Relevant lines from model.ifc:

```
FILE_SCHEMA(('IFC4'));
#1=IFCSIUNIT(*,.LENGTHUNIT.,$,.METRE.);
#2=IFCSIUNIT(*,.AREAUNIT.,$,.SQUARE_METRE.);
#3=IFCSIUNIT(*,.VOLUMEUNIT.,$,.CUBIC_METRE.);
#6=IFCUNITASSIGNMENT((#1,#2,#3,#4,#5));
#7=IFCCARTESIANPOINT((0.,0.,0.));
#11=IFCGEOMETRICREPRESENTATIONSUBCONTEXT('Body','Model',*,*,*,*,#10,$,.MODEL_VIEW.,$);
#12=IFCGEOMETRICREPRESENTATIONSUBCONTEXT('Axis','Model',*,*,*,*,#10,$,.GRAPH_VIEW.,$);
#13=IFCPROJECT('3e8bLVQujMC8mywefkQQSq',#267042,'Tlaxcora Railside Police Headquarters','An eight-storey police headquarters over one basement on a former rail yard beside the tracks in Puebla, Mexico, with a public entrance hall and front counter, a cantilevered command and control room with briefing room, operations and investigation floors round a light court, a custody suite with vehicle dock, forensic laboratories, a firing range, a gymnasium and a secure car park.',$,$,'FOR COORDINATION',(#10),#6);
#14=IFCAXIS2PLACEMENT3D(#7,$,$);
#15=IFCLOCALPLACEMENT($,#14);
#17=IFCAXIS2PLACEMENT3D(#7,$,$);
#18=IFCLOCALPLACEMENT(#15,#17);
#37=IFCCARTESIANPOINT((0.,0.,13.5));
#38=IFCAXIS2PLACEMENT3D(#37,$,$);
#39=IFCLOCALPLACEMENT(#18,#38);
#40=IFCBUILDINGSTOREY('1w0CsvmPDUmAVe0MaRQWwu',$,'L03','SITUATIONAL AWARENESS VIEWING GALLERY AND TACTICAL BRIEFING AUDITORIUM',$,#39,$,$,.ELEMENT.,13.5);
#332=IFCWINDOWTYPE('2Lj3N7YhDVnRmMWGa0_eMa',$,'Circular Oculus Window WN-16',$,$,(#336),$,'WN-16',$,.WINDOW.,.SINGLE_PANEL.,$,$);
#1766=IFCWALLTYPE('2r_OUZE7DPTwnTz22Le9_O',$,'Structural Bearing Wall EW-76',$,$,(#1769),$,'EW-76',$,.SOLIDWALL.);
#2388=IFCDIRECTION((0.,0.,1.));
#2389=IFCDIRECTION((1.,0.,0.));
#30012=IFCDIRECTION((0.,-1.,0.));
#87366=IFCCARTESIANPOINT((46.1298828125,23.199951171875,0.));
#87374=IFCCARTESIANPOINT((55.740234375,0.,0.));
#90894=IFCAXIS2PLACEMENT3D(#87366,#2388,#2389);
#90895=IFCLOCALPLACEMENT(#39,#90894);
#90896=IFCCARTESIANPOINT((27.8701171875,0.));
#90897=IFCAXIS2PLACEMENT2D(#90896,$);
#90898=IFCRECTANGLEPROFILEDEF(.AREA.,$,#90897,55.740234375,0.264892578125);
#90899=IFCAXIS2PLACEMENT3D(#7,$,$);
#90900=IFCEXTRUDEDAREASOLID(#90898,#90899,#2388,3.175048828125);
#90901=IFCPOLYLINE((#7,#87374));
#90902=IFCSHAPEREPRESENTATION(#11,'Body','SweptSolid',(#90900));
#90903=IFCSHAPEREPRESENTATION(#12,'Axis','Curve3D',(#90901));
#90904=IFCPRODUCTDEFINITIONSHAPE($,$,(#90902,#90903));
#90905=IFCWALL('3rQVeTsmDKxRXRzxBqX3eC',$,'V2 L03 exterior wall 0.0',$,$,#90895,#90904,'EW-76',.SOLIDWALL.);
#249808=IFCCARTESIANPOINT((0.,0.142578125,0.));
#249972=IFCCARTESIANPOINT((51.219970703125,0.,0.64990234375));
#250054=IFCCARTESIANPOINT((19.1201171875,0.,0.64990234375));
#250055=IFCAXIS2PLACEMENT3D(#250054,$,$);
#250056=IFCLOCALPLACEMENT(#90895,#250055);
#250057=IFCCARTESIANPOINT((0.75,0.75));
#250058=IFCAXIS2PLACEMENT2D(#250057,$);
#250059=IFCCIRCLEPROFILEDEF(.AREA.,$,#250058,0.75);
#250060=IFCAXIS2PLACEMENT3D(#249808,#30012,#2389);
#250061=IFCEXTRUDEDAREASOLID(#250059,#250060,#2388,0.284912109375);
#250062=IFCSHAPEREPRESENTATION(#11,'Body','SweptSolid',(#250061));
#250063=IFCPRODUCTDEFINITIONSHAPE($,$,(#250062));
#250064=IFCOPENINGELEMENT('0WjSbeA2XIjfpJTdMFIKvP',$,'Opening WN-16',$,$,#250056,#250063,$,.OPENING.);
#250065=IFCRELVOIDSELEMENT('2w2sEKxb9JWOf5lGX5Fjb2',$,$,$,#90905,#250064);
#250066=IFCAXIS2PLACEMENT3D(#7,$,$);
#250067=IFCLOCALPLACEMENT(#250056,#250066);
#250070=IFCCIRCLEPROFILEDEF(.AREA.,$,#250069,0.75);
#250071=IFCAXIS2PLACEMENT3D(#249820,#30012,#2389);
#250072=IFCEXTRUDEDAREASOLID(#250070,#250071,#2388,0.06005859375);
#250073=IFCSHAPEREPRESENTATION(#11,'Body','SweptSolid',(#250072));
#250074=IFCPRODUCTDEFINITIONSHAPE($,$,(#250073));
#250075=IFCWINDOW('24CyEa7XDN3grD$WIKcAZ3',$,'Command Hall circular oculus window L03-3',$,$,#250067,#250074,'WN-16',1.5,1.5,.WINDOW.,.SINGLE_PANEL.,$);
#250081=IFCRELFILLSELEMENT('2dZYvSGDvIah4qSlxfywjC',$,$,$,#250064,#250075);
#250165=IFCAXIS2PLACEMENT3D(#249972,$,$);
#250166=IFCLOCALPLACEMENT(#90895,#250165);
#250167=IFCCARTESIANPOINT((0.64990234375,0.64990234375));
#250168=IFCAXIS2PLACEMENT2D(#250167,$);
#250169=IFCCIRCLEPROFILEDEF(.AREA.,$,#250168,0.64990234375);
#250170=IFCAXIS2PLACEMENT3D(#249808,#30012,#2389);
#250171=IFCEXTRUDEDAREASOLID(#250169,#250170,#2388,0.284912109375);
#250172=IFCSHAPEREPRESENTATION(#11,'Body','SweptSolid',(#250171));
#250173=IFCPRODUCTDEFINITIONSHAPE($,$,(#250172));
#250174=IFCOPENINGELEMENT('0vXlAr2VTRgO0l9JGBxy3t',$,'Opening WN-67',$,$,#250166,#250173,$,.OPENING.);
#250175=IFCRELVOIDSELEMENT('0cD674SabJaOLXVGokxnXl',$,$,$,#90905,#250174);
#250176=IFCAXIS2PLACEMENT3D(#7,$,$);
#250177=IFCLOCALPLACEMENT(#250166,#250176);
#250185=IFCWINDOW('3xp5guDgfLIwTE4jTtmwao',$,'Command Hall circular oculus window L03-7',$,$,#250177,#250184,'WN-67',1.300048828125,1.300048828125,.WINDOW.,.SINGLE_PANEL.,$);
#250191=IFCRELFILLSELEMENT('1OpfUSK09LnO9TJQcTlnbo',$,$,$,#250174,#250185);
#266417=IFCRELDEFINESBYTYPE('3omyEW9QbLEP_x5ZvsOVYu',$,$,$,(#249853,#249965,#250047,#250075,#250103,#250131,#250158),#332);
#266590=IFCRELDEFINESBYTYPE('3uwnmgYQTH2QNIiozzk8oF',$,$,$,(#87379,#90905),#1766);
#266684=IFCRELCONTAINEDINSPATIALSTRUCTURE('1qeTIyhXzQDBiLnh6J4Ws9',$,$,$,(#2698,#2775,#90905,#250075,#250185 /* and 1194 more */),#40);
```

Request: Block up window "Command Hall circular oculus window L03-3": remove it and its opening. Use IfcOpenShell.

```python
import ifcopenshell
import ifcopenshell.api.feature
import ifcopenshell.api.root
import ifcopenshell.geom
import ifcopenshell.util.shape

model = ifcopenshell.open("model.ifc")
settings = ifcopenshell.geom.settings()


def volume(element):
    """Net volume in cubic metres, openings subtracted."""
    shape = ifcopenshell.geom.create_shape(settings, element)
    return ifcopenshell.util.shape.get_volume(shape.geometry)


window = model.by_id(250075)
opening = window.FillsVoids[0].RelatingOpeningElement
wall = opening.VoidsElements[0].RelatingBuildingElement
before = volume(wall)

ifcopenshell.api.root.remove_product(model, product=window)
ifcopenshell.api.feature.remove_feature(model, feature=opening)

after = volume(wall)

print(f"wall volume {before:.3f} -> {after:.3f} m3")

model.write("model_edited.ifc")
```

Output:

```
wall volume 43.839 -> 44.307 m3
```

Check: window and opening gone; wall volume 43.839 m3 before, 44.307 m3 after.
